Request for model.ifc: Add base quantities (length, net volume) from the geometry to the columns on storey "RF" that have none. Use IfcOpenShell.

First a look at what the model holds.

```python
import ifcopenshell
import ifcopenshell.util.element
import ifcopenshell.util.unit

model = ifcopenshell.open("model.ifc")
print(model.schema)
for unit_type in ("LENGTHUNIT", "AREAUNIT", "VOLUMEUNIT"):
    print(unit_type, ifcopenshell.util.unit.calculate_unit_scale(model, unit_type))
storey = next(s for s in model.by_type("IfcBuildingStorey") if s.Name == "RF")
columns = [e for e in ifcopenshell.util.element.get_decomposition(storey) if e.is_a("IfcColumn")]
for e in sorted(columns, key=lambda e: e.id()):
    print(e.id(), e.is_a(), e.Name, list(ifcopenshell.util.element.get_psets(e, qtos_only=True)), sep=" | ")
```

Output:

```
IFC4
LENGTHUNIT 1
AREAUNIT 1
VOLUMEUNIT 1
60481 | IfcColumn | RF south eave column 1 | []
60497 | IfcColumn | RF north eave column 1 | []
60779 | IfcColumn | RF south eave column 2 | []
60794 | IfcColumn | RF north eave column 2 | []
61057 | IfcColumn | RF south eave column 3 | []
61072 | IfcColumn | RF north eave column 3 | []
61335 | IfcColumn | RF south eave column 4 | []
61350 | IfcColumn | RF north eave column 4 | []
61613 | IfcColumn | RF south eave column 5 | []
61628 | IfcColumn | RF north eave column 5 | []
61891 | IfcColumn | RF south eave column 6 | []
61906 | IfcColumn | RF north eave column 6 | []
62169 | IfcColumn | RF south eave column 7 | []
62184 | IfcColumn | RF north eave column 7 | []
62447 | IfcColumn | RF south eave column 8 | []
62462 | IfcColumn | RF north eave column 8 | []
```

```python
import ifcopenshell
import ifcopenshell.api.pset
import ifcopenshell.geom
import ifcopenshell.util.element
import ifcopenshell.util.shape
import ifcopenshell.util.unit

model = ifcopenshell.open("model.ifc")
unit_scale = ifcopenshell.util.unit.calculate_unit_scale(model)
volume_scale = ifcopenshell.util.unit.calculate_unit_scale(model, "VOLUMEUNIT")
settings = ifcopenshell.geom.settings()

storey = next(s for s in model.by_type("IfcBuildingStorey") if s.Name == "RF")
columns = [e for e in ifcopenshell.util.element.get_decomposition(storey) if e.is_a("IfcColumn")]

for e in sorted(columns, key=lambda e: e.id()):
    if ifcopenshell.util.element.get_psets(e, qtos_only=True, should_inherit=False):
        continue
    # Geometry comes back in metres, in the element's own axes.
    shape = ifcopenshell.geom.create_shape(settings, e)
    values = {
        "Length": ifcopenshell.util.shape.get_z(shape.geometry) / unit_scale,
        "NetVolume": ifcopenshell.util.shape.get_volume(shape.geometry) / volume_scale,
    }
    qto = ifcopenshell.api.pset.add_qto(model, product=e, name="Qto_ColumnBaseQuantities")
    ifcopenshell.api.pset.edit_qto(model, qto=qto, properties=values)
    print(e.id(), {k: round(v, 3) for k, v in values.items()})

model.write("model_edited.ifc")
```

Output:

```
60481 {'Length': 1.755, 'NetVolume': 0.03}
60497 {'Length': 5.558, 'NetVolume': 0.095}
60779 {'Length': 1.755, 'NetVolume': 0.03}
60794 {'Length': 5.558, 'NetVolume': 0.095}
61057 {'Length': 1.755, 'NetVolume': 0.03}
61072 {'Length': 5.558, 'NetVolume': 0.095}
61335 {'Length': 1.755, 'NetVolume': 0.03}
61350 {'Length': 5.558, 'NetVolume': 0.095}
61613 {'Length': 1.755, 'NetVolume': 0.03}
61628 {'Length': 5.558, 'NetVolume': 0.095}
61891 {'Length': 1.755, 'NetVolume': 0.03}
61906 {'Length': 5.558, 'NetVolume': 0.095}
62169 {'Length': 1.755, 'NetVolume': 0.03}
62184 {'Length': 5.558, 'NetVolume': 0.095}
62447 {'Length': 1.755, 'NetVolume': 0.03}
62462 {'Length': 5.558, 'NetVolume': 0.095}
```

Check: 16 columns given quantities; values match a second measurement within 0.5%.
